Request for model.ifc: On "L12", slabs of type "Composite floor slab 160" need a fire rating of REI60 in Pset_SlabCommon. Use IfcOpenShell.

First a look at what the model holds.

```python
import ifcopenshell
import ifcopenshell.util.element

model = ifcopenshell.open("model.ifc")
print(model.schema)
storey = next(s for s in model.by_type("IfcBuildingStorey") if s.Name == "L12")
slabs = [e for e in ifcopenshell.util.element.get_decomposition(storey) if e.is_a("IfcSlab")]
seen = {}
for e in slabs:
    element_type = ifcopenshell.util.element.get_type(e)
    key = (element_type.Name if element_type != e and element_type else None, ifcopenshell.util.element.get_pset(e, "Pset_SlabCommon", "FireRating"))
    seen[key] = seen.get(key, 0) + 1
for (name, value), count in sorted(seen.items(), key=str):
    print(count, "x", name, "|", value)
```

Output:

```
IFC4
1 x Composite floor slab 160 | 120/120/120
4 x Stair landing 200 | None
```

```python
import ifcopenshell
import ifcopenshell.api.pset
import ifcopenshell.util.element

model = ifcopenshell.open("model.ifc")

storey = next(s for s in model.by_type("IfcBuildingStorey") if s.Name == "L12")
slabs = [e for e in ifcopenshell.util.element.get_decomposition(storey) if e.is_a("IfcSlab")]

count = 0
for e in slabs:
    element_type = ifcopenshell.util.element.get_type(e)
    if element_type in (None, e) or element_type.Name != "Composite floor slab 160":
        continue
    found = ifcopenshell.util.element.get_pset(e, "Pset_SlabCommon", should_inherit=False)
    if found:
        pset = model.by_id(found["id"])
        if len(ifcopenshell.util.element.get_elements_by_pset(pset)) > 1:
            pset = ifcopenshell.api.pset.unshare_pset(model, products=[e], pset=pset)[0]
    else:
        pset = ifcopenshell.api.pset.add_pset(model, product=e, name="Pset_SlabCommon")
    ifcopenshell.api.pset.edit_pset(model, pset=pset, properties={"FireRating": "REI60"})
    count += 1

print(count, "slabs updated")

model.write("model_updated.ifc")
```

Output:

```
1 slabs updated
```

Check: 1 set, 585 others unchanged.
